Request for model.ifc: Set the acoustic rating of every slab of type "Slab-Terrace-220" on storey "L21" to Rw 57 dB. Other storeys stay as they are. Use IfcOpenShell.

First a look at what the model holds.

```python
import ifcopenshell
import ifcopenshell.util.element

model = ifcopenshell.open("model.ifc")
print(model.schema)
storey = next(s for s in model.by_type("IfcBuildingStorey") if s.Name == "L21")
slabs = [e for e in ifcopenshell.util.element.get_decomposition(storey) if e.is_a("IfcSlab")]
seen = {}
for e in slabs:
    element_type = ifcopenshell.util.element.get_type(e)
    key = (element_type.Name if element_type != e and element_type else None, ifcopenshell.util.element.get_pset(e, "Pset_SlabCommon", "AcousticRating"))
    seen[key] = seen.get(key, 0) + 1
for (name, value), count in sorted(seen.items(), key=str):
    print(count, "x", name, "|", value)
```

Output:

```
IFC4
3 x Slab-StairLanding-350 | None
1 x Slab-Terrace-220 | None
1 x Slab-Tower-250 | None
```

```python
import ifcopenshell
import ifcopenshell.api.pset
import ifcopenshell.util.element

model = ifcopenshell.open("model.ifc")

storey = next(s for s in model.by_type("IfcBuildingStorey") if s.Name == "L21")
slabs = [e for e in ifcopenshell.util.element.get_decomposition(storey) if e.is_a("IfcSlab")]

count = 0
for e in slabs:
    element_type = ifcopenshell.util.element.get_type(e)
    if element_type in (None, e) or element_type.Name != "Slab-Terrace-220":
        continue
    found = ifcopenshell.util.element.get_pset(e, "Pset_SlabCommon", should_inherit=False)
    if found:
        pset = model.by_id(found["id"])
        if len(ifcopenshell.util.element.get_elements_by_pset(pset)) > 1:
            pset = ifcopenshell.api.pset.unshare_pset(model, products=[e], pset=pset)[0]
    else:
        pset = ifcopenshell.api.pset.add_pset(model, product=e, name="Pset_SlabCommon")
    ifcopenshell.api.pset.edit_pset(model, pset=pset, properties={"AcousticRating": "Rw 57 dB"})
    count += 1

print(count, "slabs updated")

model.write("model_edited.ifc")
```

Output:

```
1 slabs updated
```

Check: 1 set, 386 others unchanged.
